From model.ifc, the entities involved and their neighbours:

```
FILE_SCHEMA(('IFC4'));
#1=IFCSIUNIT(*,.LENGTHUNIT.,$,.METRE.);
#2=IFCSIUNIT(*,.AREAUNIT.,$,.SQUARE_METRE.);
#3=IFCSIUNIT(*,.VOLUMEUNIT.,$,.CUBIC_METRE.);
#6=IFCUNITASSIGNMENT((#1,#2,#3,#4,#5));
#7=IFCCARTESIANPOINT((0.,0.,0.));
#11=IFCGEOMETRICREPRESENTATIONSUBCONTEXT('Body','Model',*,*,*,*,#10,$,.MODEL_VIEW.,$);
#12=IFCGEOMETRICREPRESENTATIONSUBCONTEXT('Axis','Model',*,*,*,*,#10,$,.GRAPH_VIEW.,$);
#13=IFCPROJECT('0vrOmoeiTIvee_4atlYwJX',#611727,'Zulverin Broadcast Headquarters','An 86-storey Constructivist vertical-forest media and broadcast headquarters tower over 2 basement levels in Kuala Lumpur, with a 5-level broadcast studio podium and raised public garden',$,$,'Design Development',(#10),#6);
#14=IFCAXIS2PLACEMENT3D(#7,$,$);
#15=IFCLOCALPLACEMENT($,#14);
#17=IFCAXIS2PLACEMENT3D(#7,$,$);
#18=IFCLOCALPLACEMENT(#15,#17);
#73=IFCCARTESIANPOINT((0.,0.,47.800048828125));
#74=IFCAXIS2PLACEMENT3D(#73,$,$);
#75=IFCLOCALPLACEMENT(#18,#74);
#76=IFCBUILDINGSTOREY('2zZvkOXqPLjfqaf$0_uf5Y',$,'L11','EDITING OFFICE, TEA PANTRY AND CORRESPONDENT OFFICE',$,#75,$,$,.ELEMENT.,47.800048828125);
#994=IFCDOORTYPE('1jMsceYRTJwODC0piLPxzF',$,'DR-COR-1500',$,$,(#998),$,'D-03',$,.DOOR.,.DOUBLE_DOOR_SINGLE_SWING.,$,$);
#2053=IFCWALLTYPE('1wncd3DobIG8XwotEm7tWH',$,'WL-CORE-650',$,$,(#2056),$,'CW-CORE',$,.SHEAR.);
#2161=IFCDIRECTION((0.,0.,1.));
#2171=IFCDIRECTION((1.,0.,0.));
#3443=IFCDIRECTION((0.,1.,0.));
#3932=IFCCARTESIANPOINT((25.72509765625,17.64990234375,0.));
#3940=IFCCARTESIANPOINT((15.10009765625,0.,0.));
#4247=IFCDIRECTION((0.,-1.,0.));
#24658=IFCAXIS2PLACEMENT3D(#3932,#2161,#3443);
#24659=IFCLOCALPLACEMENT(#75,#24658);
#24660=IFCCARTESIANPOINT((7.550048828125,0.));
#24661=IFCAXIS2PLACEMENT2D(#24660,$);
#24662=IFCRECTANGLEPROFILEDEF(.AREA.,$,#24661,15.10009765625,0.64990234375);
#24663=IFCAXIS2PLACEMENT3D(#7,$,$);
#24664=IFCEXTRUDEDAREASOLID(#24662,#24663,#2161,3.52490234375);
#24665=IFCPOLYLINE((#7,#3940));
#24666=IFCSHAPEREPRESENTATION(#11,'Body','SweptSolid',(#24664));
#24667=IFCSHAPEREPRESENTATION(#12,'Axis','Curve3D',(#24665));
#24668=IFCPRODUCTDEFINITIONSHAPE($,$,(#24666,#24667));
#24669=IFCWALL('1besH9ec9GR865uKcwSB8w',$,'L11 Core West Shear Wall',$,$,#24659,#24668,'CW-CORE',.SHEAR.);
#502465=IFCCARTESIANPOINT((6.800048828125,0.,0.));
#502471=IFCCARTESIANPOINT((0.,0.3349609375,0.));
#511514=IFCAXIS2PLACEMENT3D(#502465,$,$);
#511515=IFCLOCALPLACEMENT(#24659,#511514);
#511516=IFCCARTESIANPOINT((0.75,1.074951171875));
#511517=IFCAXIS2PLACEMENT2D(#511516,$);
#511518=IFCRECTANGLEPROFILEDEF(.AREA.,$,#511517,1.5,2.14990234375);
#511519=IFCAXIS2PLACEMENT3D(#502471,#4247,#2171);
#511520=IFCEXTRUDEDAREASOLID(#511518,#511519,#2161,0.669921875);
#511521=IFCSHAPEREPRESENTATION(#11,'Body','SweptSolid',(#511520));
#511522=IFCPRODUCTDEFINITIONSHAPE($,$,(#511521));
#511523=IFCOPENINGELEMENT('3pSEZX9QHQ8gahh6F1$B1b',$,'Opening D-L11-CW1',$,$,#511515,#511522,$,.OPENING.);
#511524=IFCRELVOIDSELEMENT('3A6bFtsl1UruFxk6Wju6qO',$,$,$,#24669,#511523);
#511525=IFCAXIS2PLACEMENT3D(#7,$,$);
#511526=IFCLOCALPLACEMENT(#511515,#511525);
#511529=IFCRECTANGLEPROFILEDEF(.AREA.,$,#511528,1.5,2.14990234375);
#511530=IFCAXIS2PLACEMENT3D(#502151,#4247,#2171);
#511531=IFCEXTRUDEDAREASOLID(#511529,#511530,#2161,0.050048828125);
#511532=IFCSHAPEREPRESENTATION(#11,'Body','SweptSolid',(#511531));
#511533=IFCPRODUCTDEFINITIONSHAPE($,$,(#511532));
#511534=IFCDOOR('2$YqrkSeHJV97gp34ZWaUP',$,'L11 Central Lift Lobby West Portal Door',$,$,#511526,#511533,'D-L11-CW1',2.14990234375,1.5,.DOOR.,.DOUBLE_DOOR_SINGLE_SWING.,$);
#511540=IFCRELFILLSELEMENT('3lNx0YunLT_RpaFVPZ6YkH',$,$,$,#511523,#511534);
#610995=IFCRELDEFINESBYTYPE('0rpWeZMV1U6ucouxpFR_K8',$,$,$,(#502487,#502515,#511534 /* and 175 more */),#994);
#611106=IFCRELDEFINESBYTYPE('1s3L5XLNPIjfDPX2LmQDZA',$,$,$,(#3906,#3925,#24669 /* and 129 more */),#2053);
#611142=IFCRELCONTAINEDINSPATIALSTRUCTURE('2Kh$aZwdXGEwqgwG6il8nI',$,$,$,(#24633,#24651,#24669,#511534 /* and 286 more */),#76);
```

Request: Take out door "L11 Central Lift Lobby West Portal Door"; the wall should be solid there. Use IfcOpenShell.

```python
import ifcopenshell
import ifcopenshell.api.feature
import ifcopenshell.api.root
import ifcopenshell.geom
import ifcopenshell.util.shape

model = ifcopenshell.open("model.ifc")
settings = ifcopenshell.geom.settings()


def volume(element):
    """Net volume in cubic metres, openings subtracted."""
    shape = ifcopenshell.geom.create_shape(settings, element)
    return ifcopenshell.util.shape.get_volume(shape.geometry)


door = model.by_guid("2$YqrkSeHJV97gp34ZWaUP")
opening = door.FillsVoids[0].RelatingOpeningElement
wall = opening.VoidsElements[0].RelatingBuildingElement
before = volume(wall)

ifcopenshell.api.root.remove_product(model, product=door)
ifcopenshell.api.feature.remove_feature(model, feature=opening)

after = volume(wall)

print(f"wall volume {before:.3f} -> {after:.3f} m3")

model.write("model_v2.ifc")
```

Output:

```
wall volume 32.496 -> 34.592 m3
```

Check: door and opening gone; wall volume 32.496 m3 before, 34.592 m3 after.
